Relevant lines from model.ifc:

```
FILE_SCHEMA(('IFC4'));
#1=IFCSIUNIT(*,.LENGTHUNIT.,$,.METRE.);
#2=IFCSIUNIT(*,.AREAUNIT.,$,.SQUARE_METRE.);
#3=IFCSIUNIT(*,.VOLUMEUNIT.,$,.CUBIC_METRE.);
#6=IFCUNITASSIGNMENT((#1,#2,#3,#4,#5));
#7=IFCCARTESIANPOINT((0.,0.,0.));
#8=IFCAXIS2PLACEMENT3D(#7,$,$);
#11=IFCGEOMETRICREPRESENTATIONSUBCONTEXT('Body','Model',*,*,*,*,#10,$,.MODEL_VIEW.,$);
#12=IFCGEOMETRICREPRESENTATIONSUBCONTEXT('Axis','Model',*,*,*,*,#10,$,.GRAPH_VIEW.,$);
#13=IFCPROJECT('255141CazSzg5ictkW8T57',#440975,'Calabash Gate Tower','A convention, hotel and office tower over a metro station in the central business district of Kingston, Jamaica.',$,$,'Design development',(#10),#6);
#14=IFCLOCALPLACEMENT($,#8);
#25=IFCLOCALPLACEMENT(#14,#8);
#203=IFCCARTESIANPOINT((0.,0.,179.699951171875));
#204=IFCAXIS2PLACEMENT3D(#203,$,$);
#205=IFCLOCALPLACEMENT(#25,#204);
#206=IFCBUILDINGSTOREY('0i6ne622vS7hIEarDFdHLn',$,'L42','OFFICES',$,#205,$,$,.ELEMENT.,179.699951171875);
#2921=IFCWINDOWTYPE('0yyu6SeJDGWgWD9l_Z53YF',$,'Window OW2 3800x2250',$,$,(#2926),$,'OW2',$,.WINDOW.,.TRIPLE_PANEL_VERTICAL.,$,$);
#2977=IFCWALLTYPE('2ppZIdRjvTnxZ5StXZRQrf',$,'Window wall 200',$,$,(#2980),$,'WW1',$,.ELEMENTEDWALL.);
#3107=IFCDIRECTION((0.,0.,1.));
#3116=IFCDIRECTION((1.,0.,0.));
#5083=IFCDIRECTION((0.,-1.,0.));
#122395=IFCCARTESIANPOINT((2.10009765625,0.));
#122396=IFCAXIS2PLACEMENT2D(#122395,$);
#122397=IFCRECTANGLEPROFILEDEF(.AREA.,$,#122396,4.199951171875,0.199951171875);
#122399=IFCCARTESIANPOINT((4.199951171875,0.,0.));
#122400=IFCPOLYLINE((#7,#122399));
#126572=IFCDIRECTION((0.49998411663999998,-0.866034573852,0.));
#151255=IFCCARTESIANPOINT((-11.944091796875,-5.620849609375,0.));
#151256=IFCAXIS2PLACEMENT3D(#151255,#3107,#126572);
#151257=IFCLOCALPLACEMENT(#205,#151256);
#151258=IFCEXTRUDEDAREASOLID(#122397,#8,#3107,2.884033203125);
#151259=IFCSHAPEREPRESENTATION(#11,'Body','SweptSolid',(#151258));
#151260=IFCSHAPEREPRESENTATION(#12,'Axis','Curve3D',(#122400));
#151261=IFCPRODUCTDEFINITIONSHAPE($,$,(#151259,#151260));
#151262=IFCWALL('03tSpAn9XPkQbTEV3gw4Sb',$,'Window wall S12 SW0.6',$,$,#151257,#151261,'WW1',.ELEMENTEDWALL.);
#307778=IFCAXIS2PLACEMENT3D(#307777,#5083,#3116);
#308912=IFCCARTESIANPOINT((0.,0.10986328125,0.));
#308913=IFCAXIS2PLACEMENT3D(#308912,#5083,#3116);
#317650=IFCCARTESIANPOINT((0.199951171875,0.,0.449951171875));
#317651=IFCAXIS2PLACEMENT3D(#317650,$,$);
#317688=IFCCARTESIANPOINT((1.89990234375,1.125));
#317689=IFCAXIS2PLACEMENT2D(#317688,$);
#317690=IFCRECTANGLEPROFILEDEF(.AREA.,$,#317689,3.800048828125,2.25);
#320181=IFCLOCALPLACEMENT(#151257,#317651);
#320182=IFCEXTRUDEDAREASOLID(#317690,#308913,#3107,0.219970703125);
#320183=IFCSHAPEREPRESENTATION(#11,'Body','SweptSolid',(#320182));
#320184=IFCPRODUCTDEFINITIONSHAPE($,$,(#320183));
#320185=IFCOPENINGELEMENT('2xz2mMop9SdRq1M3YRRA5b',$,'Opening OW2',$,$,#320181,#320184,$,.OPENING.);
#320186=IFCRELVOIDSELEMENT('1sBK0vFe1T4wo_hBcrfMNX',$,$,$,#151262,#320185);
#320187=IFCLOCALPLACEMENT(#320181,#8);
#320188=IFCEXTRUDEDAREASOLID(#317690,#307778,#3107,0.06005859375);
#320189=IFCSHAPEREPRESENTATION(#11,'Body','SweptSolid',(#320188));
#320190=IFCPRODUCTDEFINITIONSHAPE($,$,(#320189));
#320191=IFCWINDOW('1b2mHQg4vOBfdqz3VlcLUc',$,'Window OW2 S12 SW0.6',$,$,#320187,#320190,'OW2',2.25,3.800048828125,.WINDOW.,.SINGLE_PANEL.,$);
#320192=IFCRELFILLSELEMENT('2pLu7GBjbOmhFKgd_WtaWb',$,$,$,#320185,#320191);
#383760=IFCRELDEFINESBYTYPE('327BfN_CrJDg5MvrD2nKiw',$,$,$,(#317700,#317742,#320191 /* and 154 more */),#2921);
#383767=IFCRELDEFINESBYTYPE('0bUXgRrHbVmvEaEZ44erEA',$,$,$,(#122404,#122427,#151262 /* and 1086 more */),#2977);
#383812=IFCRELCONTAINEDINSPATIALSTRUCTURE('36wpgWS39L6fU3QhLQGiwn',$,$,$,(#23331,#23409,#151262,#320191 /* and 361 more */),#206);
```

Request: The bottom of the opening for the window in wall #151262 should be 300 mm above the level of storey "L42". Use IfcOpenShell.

```python
import numpy as np
import ifcopenshell
import ifcopenshell.api.geometry
import ifcopenshell.geom
import ifcopenshell.util.element
import ifcopenshell.util.placement
import ifcopenshell.util.shape
import ifcopenshell.util.unit

model = ifcopenshell.open("model.ifc")
unit_scale = ifcopenshell.util.unit.calculate_unit_scale(model)

window = model.by_guid("1b2mHQg4vOBfdqz3VlcLUc")
opening = window.FillsVoids[0].RelatingOpeningElement
storey = ifcopenshell.util.element.get_container(window, ifc_class="IfcBuildingStorey")
level = ifcopenshell.util.placement.get_local_placement(storey.ObjectPlacement)[2, 3]

# The opening's origin need not be at the sill, so measure its lowest point.
shape = ifcopenshell.geom.create_shape(ifcopenshell.geom.settings(), opening)
bottom = ifcopenshell.util.shape.get_shape_bottom_elevation(shape, shape.geometry) / unit_scale
dz = level + 0.3 - bottom

shift = np.array([0.0, 0.0, dz])
# The window is placed relative to its opening, so it follows when the opening moves.
matrix = ifcopenshell.util.placement.get_local_placement(opening.ObjectPlacement)
matrix[:3, 3] += shift
ifcopenshell.api.geometry.edit_object_placement(
    model, product=opening, matrix=matrix, is_si=False, should_transform_children=True
)

print(f"moved by {dz * unit_scale:+.3f} m")

model.write("model_edited.ifc")
```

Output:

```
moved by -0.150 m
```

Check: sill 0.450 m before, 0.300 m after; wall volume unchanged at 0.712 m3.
